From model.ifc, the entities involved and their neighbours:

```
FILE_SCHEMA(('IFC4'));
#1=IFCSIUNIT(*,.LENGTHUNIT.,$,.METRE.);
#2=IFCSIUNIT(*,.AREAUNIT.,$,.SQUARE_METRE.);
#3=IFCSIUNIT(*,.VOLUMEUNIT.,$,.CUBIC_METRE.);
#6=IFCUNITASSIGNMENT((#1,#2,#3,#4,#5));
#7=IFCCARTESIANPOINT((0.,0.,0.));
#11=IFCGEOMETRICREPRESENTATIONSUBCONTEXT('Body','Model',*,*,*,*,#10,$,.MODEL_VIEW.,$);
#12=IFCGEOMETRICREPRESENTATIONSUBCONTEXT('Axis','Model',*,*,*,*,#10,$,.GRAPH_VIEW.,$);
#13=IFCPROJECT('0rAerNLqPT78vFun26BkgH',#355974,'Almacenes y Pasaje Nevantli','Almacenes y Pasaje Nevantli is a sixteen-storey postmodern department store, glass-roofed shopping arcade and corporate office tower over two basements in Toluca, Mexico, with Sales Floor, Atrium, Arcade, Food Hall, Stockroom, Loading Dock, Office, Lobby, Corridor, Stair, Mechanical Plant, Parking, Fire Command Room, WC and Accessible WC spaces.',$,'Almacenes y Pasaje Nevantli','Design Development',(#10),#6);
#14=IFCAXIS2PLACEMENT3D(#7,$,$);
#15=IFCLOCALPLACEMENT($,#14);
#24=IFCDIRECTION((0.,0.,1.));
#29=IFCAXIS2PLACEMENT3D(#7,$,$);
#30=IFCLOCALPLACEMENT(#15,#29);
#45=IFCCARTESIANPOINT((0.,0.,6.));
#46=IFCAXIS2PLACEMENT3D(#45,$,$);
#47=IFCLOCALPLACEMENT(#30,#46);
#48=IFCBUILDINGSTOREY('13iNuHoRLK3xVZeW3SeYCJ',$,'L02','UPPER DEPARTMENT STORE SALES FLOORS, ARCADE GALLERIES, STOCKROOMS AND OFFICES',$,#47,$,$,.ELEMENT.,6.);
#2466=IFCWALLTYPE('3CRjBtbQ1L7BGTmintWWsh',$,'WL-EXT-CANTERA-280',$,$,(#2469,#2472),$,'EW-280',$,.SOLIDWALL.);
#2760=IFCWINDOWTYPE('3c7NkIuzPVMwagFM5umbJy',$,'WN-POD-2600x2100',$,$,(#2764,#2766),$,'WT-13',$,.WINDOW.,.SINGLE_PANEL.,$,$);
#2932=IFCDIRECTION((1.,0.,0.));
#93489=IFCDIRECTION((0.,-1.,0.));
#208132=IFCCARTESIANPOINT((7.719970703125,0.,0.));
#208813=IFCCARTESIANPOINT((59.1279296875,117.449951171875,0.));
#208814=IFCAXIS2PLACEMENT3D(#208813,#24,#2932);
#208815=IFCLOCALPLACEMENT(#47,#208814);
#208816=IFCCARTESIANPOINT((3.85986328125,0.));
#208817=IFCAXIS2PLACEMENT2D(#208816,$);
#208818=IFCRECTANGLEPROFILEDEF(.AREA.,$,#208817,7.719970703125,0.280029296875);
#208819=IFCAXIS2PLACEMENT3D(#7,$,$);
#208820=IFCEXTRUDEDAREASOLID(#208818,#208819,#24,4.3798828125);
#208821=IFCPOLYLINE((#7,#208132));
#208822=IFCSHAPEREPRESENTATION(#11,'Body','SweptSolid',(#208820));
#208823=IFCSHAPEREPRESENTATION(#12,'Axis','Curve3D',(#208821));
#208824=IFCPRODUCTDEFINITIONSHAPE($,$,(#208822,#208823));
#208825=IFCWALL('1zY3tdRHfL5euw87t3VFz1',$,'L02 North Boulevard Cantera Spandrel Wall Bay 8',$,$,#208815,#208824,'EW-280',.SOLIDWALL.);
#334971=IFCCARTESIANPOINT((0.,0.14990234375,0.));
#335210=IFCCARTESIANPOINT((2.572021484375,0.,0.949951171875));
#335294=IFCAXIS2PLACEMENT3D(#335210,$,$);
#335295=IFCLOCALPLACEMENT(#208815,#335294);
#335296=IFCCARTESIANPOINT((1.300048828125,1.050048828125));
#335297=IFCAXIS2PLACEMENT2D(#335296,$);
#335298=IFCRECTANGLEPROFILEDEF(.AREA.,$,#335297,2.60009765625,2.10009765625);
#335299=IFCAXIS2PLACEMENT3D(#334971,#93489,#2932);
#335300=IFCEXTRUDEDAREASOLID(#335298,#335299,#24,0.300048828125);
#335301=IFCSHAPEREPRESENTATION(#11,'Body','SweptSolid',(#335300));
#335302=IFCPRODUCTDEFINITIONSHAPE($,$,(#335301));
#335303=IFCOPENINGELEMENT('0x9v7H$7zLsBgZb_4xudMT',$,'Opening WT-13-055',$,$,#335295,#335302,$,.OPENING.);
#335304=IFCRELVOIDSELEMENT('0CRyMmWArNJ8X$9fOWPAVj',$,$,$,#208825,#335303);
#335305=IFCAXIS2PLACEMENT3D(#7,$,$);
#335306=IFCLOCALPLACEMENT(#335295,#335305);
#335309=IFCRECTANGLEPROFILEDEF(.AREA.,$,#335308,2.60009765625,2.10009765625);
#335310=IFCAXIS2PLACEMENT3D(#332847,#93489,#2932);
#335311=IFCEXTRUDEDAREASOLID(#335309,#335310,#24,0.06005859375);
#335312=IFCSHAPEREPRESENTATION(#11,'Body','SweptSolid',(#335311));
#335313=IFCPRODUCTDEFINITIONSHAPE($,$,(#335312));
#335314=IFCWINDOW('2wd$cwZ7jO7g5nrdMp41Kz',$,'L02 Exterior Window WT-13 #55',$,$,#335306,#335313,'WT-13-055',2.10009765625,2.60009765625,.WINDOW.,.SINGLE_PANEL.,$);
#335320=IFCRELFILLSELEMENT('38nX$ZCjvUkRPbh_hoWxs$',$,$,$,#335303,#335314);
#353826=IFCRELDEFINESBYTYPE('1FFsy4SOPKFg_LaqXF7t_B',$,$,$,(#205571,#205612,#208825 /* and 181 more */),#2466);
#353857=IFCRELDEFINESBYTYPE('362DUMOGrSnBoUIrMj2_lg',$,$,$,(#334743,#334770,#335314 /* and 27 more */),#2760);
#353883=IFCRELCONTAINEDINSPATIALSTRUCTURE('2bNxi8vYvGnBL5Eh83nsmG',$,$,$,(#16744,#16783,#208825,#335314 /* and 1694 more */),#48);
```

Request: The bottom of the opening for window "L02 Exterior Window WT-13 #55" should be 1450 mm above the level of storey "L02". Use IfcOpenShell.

```python
import numpy as np
import ifcopenshell
import ifcopenshell.api.geometry
import ifcopenshell.geom
import ifcopenshell.util.element
import ifcopenshell.util.placement
import ifcopenshell.util.shape
import ifcopenshell.util.unit

model = ifcopenshell.open("model.ifc")
unit_scale = ifcopenshell.util.unit.calculate_unit_scale(model)

window = model.by_guid("2wd$cwZ7jO7g5nrdMp41Kz")
opening = window.FillsVoids[0].RelatingOpeningElement
storey = ifcopenshell.util.element.get_container(window, ifc_class="IfcBuildingStorey")
level = ifcopenshell.util.placement.get_local_placement(storey.ObjectPlacement)[2, 3]

# The opening's origin need not be at the sill, so measure its lowest point.
shape = ifcopenshell.geom.create_shape(ifcopenshell.geom.settings(), opening)
bottom = ifcopenshell.util.shape.get_shape_bottom_elevation(shape, shape.geometry) / unit_scale
dz = level + 1.45 / unit_scale - bottom

shift = np.array([0.0, 0.0, dz])
# The window is placed relative to its opening, so it follows when the opening moves.
matrix = ifcopenshell.util.placement.get_local_placement(opening.ObjectPlacement)
matrix[:3, 3] += shift
ifcopenshell.api.geometry.edit_object_placement(
    model, product=opening, matrix=matrix, is_si=False, should_transform_children=True
)

print(f"moved by {dz * unit_scale:+.3f} m")

model.write("model_rev.ifc")
```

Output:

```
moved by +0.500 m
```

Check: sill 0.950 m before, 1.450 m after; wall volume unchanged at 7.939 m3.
